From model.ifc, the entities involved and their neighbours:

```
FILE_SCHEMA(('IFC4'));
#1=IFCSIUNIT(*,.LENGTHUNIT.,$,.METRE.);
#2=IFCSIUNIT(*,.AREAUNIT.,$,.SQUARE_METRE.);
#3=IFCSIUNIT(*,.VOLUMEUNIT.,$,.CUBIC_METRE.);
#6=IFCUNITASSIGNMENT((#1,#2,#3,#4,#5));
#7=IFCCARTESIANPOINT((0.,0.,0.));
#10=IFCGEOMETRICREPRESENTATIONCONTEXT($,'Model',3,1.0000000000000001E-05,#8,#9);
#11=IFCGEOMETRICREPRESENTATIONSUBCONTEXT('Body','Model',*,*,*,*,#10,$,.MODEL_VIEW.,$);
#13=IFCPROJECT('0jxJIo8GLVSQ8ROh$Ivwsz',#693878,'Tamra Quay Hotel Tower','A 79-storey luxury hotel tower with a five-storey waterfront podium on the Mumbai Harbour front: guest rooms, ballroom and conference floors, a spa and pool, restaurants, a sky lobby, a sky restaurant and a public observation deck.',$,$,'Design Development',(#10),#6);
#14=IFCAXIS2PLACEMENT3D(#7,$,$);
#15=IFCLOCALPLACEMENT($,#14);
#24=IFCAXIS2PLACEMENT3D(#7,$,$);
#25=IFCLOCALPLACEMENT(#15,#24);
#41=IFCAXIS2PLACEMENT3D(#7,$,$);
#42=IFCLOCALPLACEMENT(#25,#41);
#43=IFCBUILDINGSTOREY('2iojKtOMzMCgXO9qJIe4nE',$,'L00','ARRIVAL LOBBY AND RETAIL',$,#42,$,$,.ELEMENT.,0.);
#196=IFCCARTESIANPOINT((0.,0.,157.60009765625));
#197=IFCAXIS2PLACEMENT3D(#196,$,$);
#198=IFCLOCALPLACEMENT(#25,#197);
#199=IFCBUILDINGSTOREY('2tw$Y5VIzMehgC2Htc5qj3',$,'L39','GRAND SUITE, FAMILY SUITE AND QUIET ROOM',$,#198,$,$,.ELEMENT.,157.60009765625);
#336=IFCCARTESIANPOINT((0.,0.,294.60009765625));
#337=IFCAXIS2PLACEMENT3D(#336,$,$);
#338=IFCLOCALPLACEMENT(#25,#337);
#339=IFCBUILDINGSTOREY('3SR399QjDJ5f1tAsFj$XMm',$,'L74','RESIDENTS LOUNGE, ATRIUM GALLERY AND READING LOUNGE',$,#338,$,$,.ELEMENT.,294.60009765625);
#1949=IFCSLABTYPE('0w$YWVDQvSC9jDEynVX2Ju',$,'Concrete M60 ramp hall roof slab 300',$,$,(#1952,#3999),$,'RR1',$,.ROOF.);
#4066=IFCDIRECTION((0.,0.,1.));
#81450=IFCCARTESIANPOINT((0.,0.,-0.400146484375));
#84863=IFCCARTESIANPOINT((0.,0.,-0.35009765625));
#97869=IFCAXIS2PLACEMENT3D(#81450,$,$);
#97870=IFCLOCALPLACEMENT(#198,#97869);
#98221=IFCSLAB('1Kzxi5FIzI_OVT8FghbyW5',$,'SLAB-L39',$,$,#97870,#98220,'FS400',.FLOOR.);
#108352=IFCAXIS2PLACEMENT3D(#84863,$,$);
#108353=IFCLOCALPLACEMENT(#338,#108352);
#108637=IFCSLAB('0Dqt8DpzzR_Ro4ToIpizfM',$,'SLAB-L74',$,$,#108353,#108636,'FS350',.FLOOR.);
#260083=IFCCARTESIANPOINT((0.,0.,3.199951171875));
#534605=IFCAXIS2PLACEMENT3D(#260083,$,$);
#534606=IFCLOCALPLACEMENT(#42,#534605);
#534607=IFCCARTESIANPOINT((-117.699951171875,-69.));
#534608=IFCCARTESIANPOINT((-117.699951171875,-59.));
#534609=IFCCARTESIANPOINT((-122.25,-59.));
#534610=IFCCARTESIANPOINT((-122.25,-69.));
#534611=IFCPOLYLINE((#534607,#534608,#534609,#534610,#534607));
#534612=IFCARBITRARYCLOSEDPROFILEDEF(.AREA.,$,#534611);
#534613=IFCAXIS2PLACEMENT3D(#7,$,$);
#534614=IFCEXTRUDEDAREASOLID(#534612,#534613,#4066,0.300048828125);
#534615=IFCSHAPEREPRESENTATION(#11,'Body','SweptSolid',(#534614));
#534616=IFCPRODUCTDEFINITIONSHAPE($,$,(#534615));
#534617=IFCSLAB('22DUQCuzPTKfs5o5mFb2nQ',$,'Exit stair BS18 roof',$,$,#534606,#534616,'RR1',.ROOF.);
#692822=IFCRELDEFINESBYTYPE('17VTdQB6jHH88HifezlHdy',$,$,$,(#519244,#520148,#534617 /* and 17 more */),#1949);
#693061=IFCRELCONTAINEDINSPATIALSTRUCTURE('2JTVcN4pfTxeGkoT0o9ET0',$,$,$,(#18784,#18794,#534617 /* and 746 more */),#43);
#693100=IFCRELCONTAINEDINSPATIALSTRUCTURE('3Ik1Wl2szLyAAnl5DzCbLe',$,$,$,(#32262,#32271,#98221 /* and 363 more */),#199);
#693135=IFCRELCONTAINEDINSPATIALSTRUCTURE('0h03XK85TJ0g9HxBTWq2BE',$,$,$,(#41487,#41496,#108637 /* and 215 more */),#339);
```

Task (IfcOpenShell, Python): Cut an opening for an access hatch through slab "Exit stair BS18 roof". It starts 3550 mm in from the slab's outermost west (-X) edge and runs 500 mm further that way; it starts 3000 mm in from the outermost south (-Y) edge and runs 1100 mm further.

```python
import numpy as np
import ifcopenshell
import ifcopenshell.api.feature
import ifcopenshell.api.geometry
import ifcopenshell.api.root
import ifcopenshell.geom
import ifcopenshell.util.placement
import ifcopenshell.util.representation
import ifcopenshell.util.shape
import ifcopenshell.util.unit

model = ifcopenshell.open("model.ifc")
unit_scale = ifcopenshell.util.unit.calculate_unit_scale(model)
settings = ifcopenshell.geom.settings()


def volume(element):
    """Net volume in cubic metres, openings subtracted."""
    shape = ifcopenshell.geom.create_shape(settings, element)
    return ifcopenshell.util.shape.get_volume(shape.geometry)


slab = model.by_guid("22DUQCuzPTKfs5o5mFb2nQ")
before = volume(slab)

# Extent in the slab's own axes, in metres. The edges named are its -X and -Y sides.
slab_shape = ifcopenshell.geom.create_shape(settings, slab)
vertices = ifcopenshell.util.shape.get_vertices(slab_shape.geometry)
x_min, y_min, bottom = vertices.min(axis=0)
top = vertices[:, 2].max()

opening = ifcopenshell.api.root.create_entity(model, ifc_class="IfcOpeningElement", name="Access hatch opening", predefined_type="OPENING")
context = ifcopenshell.util.representation.get_context(model, "Model", "Body", "MODEL_VIEW")
width, depth = 0.5, 1.1
outline = [(0.0, 0.0), (width, 0.0), (width, depth), (0.0, depth), (0.0, 0.0)]
# Overshoot both faces by 50 mm so the cut is clean.
shape = ifcopenshell.api.geometry.add_slab_representation(
    model, context=context, depth=top - bottom + 0.1, polyline=outline
)
ifcopenshell.api.geometry.assign_representation(model, product=opening, representation=shape)

matrix = ifcopenshell.util.placement.get_local_placement(slab.ObjectPlacement)
matrix[:, 3] = matrix @ np.append(np.array([x_min + 3.55, y_min + 3, bottom - 0.05]) / unit_scale, 1.0)
ifcopenshell.api.geometry.edit_object_placement(model, product=opening, matrix=matrix, is_si=False)
ifcopenshell.api.feature.add_feature(model, feature=opening, element=slab)

after = volume(slab)

print(f"slab volume {before:.3f} -> {after:.3f} m3")

model.write("model_updated.ifc")
```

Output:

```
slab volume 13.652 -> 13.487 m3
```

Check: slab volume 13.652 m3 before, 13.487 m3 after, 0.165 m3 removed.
